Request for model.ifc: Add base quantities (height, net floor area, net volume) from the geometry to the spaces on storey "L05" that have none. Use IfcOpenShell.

First a look at what the model holds.

```python
import ifcopenshell
import ifcopenshell.util.element
import ifcopenshell.util.unit

model = ifcopenshell.open("model.ifc")
print(model.schema)
for unit_type in ("LENGTHUNIT", "AREAUNIT", "VOLUMEUNIT"):
    print(unit_type, ifcopenshell.util.unit.calculate_unit_scale(model, unit_type))
storey = next(s for s in model.by_type("IfcBuildingStorey") if s.Name == "L05")
spaces = [e for e in ifcopenshell.util.element.get_decomposition(storey) if e.is_a("IfcSpace")]
for e in sorted(spaces, key=lambda e: e.id()):
    print(e.id(), e.is_a(), e.Name, list(ifcopenshell.util.element.get_psets(e, qtos_only=True)), sep=" | ")
```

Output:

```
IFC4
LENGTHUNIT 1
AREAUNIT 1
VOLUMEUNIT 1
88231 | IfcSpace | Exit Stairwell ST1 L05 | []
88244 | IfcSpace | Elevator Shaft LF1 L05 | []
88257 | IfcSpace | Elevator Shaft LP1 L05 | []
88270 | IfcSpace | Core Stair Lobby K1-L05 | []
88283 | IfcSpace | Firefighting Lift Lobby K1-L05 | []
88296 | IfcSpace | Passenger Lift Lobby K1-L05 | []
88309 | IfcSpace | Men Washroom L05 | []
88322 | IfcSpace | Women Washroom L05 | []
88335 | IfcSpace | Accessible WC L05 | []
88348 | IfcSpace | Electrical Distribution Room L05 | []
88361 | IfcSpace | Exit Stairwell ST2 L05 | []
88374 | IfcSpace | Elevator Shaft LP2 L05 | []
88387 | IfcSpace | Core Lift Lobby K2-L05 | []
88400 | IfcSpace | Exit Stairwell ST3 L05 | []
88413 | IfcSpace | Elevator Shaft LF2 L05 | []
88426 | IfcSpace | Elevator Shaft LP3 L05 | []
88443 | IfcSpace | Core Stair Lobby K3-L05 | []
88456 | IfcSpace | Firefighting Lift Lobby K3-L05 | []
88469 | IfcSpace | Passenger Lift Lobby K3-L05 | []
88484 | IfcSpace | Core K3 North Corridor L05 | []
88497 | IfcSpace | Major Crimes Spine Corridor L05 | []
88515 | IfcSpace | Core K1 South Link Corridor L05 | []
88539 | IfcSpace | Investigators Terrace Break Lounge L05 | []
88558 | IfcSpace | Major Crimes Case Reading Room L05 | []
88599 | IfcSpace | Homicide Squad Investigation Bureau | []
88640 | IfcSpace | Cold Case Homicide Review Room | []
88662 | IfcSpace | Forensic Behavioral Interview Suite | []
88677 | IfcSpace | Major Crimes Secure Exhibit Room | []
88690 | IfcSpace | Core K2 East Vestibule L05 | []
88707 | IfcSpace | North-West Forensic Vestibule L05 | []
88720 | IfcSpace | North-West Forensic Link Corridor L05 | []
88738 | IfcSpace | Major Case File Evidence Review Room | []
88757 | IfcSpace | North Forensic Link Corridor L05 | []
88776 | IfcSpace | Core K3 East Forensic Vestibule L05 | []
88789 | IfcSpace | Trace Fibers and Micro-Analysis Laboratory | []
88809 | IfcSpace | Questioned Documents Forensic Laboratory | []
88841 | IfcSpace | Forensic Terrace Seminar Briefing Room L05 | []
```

```python
import ifcopenshell
import ifcopenshell.api.pset
import ifcopenshell.geom
import ifcopenshell.util.element
import ifcopenshell.util.shape
import ifcopenshell.util.unit

model = ifcopenshell.open("model.ifc")
unit_scale = ifcopenshell.util.unit.calculate_unit_scale(model)
area_scale = ifcopenshell.util.unit.calculate_unit_scale(model, "AREAUNIT")
volume_scale = ifcopenshell.util.unit.calculate_unit_scale(model, "VOLUMEUNIT")
settings = ifcopenshell.geom.settings()

storey = next(s for s in model.by_type("IfcBuildingStorey") if s.Name == "L05")
spaces = [e for e in ifcopenshell.util.element.get_decomposition(storey) if e.is_a("IfcSpace")]

for e in sorted(spaces, key=lambda e: e.id()):
    if ifcopenshell.util.element.get_psets(e, qtos_only=True, should_inherit=False):
        continue
    # Geometry comes back in metres, in the element's own axes.
    shape = ifcopenshell.geom.create_shape(settings, e)
    values = {
        "Height": ifcopenshell.util.shape.get_z(shape.geometry) / unit_scale,
        "NetFloorArea": ifcopenshell.util.shape.get_footprint_area(shape.geometry) / area_scale,
        "NetVolume": ifcopenshell.util.shape.get_volume(shape.geometry) / volume_scale,
    }
    qto = ifcopenshell.api.pset.add_qto(model, product=e, name="Qto_SpaceBaseQuantities")
    ifcopenshell.api.pset.edit_qto(model, qto=qto, properties=values)
    print(e.id(), {k: round(v, 3) for k, v in values.items()})

model.write("model_rev.ifc")
```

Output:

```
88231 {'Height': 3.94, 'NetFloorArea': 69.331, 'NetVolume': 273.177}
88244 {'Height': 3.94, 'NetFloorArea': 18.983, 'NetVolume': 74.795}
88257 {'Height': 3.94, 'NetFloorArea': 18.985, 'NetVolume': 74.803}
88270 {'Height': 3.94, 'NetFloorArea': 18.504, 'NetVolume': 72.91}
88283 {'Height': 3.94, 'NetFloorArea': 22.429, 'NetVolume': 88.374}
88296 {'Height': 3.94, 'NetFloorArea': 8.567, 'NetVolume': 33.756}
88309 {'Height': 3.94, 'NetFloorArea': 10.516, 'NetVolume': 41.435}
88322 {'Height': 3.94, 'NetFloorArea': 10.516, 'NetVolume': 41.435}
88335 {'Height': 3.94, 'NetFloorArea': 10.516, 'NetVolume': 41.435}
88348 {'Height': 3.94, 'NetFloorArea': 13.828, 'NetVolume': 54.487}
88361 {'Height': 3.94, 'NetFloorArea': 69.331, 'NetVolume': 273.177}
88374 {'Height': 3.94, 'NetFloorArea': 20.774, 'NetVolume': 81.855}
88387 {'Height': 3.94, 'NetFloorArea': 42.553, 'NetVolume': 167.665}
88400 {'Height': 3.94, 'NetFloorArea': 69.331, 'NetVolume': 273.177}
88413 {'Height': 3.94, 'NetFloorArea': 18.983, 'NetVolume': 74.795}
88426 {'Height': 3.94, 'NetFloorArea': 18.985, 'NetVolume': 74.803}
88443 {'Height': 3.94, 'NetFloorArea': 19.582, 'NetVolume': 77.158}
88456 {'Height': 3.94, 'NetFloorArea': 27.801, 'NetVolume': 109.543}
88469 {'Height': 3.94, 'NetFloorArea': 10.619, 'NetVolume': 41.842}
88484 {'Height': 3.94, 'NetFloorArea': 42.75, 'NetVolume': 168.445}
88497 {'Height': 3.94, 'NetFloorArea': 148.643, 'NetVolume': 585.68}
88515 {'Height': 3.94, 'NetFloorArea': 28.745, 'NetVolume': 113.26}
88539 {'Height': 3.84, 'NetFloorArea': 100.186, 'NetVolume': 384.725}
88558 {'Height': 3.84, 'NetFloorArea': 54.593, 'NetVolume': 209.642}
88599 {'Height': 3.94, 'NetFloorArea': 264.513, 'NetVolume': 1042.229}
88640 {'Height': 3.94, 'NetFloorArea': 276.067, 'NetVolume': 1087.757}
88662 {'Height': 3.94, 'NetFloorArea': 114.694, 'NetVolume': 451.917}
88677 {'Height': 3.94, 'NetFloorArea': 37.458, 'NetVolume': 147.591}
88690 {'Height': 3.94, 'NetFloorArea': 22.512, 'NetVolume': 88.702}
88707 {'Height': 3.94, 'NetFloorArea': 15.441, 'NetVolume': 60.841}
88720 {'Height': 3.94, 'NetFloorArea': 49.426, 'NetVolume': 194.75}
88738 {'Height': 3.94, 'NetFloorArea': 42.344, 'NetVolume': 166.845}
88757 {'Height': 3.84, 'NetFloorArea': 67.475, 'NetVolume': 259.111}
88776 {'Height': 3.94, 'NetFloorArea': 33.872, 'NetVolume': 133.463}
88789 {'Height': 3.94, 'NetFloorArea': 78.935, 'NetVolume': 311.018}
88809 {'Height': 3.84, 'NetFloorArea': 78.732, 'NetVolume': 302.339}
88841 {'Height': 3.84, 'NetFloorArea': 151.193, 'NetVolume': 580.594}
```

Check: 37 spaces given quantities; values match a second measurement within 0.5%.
